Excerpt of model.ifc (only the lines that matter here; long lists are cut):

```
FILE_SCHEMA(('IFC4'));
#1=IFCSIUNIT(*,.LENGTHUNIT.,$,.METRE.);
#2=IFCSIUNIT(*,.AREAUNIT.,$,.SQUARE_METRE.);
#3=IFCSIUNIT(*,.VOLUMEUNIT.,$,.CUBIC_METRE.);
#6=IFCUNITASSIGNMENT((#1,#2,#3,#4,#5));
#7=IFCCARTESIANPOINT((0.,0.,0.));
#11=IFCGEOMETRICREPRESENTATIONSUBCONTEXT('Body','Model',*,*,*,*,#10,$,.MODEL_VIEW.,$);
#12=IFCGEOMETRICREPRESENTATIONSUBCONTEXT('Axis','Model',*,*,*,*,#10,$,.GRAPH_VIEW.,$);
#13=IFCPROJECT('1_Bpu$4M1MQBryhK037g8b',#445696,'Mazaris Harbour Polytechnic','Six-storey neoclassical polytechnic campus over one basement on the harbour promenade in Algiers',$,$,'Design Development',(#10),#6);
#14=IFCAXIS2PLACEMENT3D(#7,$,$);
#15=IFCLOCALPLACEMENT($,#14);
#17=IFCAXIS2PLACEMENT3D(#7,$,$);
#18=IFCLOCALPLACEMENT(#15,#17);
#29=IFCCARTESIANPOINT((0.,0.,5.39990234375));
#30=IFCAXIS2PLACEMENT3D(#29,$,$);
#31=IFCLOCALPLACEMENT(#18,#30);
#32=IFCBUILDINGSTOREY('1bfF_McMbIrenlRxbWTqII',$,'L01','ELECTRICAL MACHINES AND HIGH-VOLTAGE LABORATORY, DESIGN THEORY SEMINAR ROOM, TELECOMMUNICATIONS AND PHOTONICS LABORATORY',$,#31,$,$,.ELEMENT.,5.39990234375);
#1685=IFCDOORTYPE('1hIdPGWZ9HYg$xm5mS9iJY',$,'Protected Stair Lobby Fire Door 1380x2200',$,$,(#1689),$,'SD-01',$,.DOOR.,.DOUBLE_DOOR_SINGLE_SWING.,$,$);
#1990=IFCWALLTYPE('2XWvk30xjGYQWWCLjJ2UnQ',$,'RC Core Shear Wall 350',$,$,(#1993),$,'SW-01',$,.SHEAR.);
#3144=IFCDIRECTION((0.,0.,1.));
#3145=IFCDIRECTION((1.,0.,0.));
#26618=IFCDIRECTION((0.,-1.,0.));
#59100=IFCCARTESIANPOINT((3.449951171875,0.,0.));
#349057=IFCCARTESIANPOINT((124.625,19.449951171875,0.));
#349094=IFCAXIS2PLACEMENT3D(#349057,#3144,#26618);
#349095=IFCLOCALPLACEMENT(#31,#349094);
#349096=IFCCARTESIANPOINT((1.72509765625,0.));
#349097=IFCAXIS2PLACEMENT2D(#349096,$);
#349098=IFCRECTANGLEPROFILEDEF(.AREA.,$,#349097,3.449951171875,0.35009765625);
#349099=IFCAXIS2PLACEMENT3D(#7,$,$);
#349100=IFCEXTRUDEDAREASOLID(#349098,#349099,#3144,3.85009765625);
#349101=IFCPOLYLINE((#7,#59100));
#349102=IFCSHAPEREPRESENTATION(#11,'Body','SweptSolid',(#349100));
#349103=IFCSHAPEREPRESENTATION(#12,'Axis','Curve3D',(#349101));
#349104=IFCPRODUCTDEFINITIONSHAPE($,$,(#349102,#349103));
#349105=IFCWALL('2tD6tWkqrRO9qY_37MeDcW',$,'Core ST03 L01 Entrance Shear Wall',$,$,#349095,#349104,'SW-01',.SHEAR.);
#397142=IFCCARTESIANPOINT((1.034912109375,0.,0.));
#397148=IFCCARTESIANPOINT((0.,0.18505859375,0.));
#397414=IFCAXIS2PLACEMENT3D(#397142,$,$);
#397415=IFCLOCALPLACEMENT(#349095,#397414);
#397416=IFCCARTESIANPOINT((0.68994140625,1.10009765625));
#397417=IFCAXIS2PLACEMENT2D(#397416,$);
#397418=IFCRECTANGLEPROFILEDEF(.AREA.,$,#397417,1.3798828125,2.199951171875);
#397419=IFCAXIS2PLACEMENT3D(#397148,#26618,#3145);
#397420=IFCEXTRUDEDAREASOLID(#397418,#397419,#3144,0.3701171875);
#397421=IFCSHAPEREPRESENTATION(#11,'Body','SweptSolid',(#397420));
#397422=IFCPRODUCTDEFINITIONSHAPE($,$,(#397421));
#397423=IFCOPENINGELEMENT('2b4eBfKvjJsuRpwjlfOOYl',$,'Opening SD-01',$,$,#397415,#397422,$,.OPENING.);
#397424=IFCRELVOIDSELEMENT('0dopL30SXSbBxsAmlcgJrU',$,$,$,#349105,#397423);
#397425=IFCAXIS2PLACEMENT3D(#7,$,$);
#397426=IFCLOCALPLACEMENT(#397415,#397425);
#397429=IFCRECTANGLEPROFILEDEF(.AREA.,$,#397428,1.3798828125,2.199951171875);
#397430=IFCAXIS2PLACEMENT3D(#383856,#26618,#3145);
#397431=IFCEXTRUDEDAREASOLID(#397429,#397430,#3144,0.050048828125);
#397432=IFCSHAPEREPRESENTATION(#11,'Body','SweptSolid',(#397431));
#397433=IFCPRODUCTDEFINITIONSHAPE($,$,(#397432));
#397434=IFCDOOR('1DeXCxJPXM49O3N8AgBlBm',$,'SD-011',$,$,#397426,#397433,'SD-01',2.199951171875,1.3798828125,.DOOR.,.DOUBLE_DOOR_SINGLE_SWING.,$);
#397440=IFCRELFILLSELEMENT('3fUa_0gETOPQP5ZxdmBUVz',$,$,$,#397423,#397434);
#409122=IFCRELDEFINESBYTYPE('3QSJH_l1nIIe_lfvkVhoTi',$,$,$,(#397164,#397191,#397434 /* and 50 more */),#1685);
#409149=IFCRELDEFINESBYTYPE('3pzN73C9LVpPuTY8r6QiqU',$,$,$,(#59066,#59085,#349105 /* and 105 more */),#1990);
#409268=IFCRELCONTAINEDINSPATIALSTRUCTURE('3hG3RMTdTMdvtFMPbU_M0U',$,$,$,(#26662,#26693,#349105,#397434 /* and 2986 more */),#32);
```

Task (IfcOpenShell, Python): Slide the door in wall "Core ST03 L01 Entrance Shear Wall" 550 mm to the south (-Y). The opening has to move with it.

```python
import ifcopenshell
import ifcopenshell.api.geometry
import ifcopenshell.util.placement

model = ifcopenshell.open("model.ifc")

door = model.by_guid("1DeXCxJPXM49O3N8AgBlBm")
opening = door.FillsVoids[0].RelatingOpeningElement
wall = opening.VoidsElements[0].RelatingBuildingElement

wall_matrix = ifcopenshell.util.placement.get_local_placement(wall.ObjectPlacement)
shift = wall_matrix[:3, 0] * 0.55
before = ifcopenshell.util.placement.get_local_placement(door.ObjectPlacement)[:3, 3].copy()

# The door is placed relative to its opening, so it follows when the opening moves.
matrix = ifcopenshell.util.placement.get_local_placement(opening.ObjectPlacement)
matrix[:3, 3] += shift
ifcopenshell.api.geometry.edit_object_placement(
    model, product=opening, matrix=matrix, is_si=False, should_transform_children=True
)

after = ifcopenshell.util.placement.get_local_placement(door.ObjectPlacement)[:3, 3]
print("door moved by", (after - before).round(3) + 0.0)

model.write("model-out.ifc")
```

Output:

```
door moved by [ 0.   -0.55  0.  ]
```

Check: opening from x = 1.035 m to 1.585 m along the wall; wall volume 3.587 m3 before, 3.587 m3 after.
